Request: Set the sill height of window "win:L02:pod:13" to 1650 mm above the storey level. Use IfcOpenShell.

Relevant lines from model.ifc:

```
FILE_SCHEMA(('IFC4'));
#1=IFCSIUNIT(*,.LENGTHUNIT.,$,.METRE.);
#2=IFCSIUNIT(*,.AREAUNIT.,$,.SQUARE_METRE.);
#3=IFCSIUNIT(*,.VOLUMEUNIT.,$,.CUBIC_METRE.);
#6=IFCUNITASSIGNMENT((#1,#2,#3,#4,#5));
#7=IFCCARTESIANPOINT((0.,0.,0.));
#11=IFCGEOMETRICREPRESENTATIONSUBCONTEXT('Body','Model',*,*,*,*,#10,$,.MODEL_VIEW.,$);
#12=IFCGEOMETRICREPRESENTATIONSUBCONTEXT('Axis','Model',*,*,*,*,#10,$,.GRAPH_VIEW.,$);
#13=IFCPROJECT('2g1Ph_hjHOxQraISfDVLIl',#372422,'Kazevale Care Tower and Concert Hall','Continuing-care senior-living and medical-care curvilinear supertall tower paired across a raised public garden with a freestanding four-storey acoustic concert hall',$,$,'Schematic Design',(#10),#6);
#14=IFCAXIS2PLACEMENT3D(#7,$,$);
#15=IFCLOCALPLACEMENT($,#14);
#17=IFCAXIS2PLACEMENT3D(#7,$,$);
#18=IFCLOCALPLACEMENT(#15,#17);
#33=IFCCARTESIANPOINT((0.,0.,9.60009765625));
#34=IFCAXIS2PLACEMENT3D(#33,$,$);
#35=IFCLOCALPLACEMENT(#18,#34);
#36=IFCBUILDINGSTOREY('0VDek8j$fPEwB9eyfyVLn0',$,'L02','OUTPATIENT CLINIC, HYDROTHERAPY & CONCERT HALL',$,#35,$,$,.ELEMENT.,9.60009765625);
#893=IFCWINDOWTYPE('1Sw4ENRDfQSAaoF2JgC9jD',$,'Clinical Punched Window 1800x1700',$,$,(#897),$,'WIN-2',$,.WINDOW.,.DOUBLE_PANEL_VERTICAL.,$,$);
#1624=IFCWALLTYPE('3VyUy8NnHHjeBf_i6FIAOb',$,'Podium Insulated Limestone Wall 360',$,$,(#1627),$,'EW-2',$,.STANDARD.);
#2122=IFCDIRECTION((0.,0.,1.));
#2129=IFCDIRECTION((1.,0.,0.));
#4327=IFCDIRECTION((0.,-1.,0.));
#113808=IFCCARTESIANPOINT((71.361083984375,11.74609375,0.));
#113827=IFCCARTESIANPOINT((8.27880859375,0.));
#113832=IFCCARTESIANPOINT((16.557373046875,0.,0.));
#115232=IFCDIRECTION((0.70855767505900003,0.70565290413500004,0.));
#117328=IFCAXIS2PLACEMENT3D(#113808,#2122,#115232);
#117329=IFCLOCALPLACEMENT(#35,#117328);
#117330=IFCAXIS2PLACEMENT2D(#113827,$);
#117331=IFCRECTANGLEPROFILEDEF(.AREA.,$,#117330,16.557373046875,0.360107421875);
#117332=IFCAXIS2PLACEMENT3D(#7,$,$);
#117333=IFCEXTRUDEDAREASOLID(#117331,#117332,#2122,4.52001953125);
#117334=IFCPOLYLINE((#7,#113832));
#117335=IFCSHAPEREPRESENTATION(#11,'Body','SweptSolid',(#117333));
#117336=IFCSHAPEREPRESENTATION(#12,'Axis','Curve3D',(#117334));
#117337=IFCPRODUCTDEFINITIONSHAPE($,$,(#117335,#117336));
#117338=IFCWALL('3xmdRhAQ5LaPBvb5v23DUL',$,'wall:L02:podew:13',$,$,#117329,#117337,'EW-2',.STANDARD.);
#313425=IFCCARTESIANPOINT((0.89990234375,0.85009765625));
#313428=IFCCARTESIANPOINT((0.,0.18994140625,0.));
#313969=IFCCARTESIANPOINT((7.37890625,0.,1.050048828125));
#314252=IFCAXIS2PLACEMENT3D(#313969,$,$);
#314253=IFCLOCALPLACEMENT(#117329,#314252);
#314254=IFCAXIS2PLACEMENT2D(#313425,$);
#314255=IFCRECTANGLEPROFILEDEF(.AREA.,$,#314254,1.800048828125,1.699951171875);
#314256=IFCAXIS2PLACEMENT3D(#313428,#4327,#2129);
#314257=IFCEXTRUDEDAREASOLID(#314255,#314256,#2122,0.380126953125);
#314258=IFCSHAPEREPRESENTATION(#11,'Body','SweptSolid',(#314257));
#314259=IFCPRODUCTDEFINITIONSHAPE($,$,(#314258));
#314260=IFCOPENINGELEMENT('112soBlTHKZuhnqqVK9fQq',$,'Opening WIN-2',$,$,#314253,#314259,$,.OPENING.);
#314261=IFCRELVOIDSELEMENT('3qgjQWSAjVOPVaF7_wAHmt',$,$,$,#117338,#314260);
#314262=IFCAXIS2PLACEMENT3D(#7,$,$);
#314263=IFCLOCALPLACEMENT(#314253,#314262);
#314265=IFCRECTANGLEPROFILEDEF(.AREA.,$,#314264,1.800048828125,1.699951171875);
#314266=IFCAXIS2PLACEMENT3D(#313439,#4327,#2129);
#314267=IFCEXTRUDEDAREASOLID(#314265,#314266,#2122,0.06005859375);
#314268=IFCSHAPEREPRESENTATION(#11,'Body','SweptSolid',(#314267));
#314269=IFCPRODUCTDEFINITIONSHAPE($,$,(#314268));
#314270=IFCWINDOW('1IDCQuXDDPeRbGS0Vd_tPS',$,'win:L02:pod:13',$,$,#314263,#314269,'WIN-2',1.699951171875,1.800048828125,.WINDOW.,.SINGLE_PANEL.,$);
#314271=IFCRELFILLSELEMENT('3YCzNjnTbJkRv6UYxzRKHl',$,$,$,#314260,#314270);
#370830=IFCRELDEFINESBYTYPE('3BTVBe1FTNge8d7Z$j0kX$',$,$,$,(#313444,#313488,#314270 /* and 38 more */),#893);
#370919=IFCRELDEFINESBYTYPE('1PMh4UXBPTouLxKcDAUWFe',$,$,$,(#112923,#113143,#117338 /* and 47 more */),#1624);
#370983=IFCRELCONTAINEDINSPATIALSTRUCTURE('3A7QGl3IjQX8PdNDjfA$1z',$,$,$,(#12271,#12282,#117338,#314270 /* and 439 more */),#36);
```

```python
import numpy as np
import ifcopenshell
import ifcopenshell.api.geometry
import ifcopenshell.geom
import ifcopenshell.util.element
import ifcopenshell.util.placement
import ifcopenshell.util.shape
import ifcopenshell.util.unit

model = ifcopenshell.open("model.ifc")
unit_scale = ifcopenshell.util.unit.calculate_unit_scale(model)

window = model.by_guid("1IDCQuXDDPeRbGS0Vd_tPS")
opening = window.FillsVoids[0].RelatingOpeningElement
storey = ifcopenshell.util.element.get_container(window, ifc_class="IfcBuildingStorey")
level = ifcopenshell.util.placement.get_local_placement(storey.ObjectPlacement)[2, 3]

# The opening's origin need not be at the sill, so measure its lowest point.
shape = ifcopenshell.geom.create_shape(ifcopenshell.geom.settings(), opening)
bottom = ifcopenshell.util.shape.get_shape_bottom_elevation(shape, shape.geometry) / unit_scale
dz = level + 1.65 / unit_scale - bottom

shift = np.array([0.0, 0.0, dz])
# The window is placed relative to its opening, so it follows when the opening moves.
matrix = ifcopenshell.util.placement.get_local_placement(opening.ObjectPlacement)
matrix[:3, 3] += shift
ifcopenshell.api.geometry.edit_object_placement(
    model, product=opening, matrix=matrix, is_si=False, should_transform_children=True
)

print(f"moved by {dz * unit_scale:+.3f} m")

model.write("model_rev.ifc")
```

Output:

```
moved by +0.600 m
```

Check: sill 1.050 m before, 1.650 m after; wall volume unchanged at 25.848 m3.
